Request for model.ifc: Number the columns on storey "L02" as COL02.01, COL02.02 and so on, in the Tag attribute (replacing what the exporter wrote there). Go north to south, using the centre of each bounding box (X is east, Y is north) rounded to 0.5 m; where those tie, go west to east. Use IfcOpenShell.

First a look at what the model holds.

```python
import ifcopenshell
import ifcopenshell.util.element
import ifcopenshell.util.placement

model = ifcopenshell.open("model.ifc")
print(model.schema)
storey = next(s for s in model.by_type("IfcBuildingStorey") if s.Name == "L02")
columns = [e for e in ifcopenshell.util.element.get_decomposition(storey) if e.is_a("IfcColumn")]
for e in sorted(columns, key=lambda e: e.id()):
    origin = ifcopenshell.util.placement.get_local_placement(e.ObjectPlacement)[:3, 3]
    print(e.id(), e.Tag, e.Name, origin.round(2) + 0.0, sep=" | ")
```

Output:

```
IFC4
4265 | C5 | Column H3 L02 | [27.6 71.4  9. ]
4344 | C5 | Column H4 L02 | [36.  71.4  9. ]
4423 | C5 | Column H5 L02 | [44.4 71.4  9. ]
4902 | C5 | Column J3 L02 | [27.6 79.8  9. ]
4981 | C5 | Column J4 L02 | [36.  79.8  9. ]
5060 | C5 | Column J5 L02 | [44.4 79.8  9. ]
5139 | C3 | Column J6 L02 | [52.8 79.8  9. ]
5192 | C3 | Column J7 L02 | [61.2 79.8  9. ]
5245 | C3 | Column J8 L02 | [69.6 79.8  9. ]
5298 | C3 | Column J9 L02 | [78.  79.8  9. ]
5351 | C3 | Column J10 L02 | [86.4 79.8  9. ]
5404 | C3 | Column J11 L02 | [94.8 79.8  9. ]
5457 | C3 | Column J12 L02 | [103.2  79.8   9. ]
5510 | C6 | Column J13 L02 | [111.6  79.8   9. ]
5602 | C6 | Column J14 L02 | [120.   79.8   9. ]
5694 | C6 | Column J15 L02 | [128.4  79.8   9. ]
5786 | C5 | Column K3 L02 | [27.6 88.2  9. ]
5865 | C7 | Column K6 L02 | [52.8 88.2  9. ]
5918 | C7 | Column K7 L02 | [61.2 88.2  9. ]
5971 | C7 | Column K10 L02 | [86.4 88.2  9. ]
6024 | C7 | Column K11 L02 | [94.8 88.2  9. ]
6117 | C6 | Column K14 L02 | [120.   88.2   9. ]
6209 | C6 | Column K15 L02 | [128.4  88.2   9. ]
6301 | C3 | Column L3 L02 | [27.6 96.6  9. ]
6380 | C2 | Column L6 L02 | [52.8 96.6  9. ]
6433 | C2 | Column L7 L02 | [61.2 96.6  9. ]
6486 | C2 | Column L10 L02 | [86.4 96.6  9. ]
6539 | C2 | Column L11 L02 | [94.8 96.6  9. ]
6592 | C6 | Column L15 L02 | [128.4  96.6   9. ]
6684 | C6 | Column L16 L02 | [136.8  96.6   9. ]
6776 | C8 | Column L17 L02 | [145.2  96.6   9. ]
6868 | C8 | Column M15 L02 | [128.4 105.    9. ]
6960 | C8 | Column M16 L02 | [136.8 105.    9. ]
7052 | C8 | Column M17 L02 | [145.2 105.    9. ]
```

```python
import ifcopenshell
import ifcopenshell.geom
import ifcopenshell.util.element
import ifcopenshell.util.shape

model = ifcopenshell.open("model.ifc")
settings = ifcopenshell.geom.settings()
settings.set("use-world-coords", True)


def centre(element):
    shape = ifcopenshell.geom.create_shape(settings, element)
    return ifcopenshell.util.shape.get_bbox_centroid(shape.geometry)


storey = next(s for s in model.by_type("IfcBuildingStorey") if s.Name == "L02")
columns = [e for e in ifcopenshell.util.element.get_decomposition(storey) if e.is_a("IfcColumn")]

# Insertion points can sit at a corner or the storey origin, so sort by the geometry (in metres).
centres = {e: centre(e) for e in columns}
columns.sort(key=lambda e: (-round(centres[e][1] / 0.5), centres[e][0]))

for i, e in enumerate(columns, start=1):
    number = f"COL02.{i:02d}"
    e.Tag = number
    print(e.id(), number)

model.write("model_rev.ifc")
```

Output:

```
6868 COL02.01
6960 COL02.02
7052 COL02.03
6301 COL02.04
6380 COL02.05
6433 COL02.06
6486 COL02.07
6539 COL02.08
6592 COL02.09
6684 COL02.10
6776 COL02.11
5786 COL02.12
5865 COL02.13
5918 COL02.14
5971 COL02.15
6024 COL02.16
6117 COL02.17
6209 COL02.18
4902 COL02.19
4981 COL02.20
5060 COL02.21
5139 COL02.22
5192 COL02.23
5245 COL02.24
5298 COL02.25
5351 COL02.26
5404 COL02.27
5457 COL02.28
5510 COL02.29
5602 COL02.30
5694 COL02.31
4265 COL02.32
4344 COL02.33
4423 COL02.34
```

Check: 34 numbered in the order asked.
